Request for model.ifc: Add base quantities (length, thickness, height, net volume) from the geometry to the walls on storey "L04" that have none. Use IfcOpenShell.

First a look at what the model holds.

```python
import ifcopenshell
import ifcopenshell.util.element
import ifcopenshell.util.unit

model = ifcopenshell.open("model.ifc")
print(model.schema)
for unit_type in ("LENGTHUNIT", "AREAUNIT", "VOLUMEUNIT"):
    print(unit_type, ifcopenshell.util.unit.calculate_unit_scale(model, unit_type))
storey = next(s for s in model.by_type("IfcBuildingStorey") if s.Name == "L04")
walls = [e for e in ifcopenshell.util.element.get_decomposition(storey) if e.is_a("IfcWall")]
for e in sorted(walls, key=lambda e: e.id()):
    print(e.id(), e.is_a(), e.Name, list(ifcopenshell.util.element.get_psets(e, qtos_only=True)), sep=" | ")
```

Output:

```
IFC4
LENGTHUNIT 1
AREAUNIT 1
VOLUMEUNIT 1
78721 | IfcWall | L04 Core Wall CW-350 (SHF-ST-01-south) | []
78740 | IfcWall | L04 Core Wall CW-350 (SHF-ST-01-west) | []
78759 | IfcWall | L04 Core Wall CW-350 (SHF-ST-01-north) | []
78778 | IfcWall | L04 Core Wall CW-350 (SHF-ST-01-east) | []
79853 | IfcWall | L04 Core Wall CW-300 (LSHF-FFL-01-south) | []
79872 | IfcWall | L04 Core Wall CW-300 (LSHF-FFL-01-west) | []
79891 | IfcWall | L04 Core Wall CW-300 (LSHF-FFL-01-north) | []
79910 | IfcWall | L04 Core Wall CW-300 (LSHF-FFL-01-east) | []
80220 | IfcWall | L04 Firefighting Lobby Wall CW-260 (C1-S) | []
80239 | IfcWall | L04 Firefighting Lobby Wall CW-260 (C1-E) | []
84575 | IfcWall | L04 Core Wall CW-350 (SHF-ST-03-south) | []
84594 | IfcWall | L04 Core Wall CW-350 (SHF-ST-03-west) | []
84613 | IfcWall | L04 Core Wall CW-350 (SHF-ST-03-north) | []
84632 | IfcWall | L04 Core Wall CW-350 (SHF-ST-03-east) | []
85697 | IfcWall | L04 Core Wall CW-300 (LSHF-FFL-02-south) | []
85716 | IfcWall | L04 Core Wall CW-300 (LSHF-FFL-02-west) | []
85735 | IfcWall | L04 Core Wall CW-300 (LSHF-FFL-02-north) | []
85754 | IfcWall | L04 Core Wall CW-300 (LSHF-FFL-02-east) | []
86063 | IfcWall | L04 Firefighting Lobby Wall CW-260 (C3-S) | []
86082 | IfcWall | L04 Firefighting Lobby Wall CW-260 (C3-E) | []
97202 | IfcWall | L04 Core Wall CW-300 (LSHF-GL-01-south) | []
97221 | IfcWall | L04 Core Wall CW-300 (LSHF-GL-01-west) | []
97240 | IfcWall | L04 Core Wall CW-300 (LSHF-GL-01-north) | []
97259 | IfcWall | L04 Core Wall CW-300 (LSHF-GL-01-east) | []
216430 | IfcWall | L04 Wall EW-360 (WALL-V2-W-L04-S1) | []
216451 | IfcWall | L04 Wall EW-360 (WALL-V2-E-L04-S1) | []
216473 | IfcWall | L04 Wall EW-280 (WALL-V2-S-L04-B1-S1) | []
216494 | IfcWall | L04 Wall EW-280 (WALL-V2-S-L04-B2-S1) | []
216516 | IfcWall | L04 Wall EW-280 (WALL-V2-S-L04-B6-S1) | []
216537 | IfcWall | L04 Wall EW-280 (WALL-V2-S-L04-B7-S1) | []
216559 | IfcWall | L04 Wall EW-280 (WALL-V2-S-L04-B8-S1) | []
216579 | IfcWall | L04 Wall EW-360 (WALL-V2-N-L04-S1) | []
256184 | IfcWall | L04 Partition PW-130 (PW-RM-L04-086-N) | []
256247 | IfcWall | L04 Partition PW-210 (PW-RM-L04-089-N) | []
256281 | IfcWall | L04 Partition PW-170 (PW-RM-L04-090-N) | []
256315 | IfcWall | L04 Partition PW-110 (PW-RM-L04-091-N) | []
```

```python
import ifcopenshell
import ifcopenshell.api.pset
import ifcopenshell.geom
import ifcopenshell.util.element
import ifcopenshell.util.shape
import ifcopenshell.util.unit

model = ifcopenshell.open("model.ifc")
unit_scale = ifcopenshell.util.unit.calculate_unit_scale(model)
volume_scale = ifcopenshell.util.unit.calculate_unit_scale(model, "VOLUMEUNIT")
settings = ifcopenshell.geom.settings()

storey = next(s for s in model.by_type("IfcBuildingStorey") if s.Name == "L04")
walls = [e for e in ifcopenshell.util.element.get_decomposition(storey) if e.is_a("IfcWall")]

for e in sorted(walls, key=lambda e: e.id()):
    if ifcopenshell.util.element.get_psets(e, qtos_only=True, should_inherit=False):
        continue
    # Geometry comes back in metres, in the element's own axes.
    shape = ifcopenshell.geom.create_shape(settings, e)
    values = {
        "Length": ifcopenshell.util.shape.get_x(shape.geometry) / unit_scale,
        "Width": ifcopenshell.util.shape.get_y(shape.geometry) / unit_scale,
        "Height": ifcopenshell.util.shape.get_z(shape.geometry) / unit_scale,
        "NetVolume": ifcopenshell.util.shape.get_volume(shape.geometry) / volume_scale,
    }
    qto = ifcopenshell.api.pset.add_qto(model, product=e, name="Qto_WallBaseQuantities")
    ifcopenshell.api.pset.edit_qto(model, qto=qto, properties=values)
    print(e.id(), {k: round(v, 3) for k, v in values.items()})

model.write("model_rev.ifc")
```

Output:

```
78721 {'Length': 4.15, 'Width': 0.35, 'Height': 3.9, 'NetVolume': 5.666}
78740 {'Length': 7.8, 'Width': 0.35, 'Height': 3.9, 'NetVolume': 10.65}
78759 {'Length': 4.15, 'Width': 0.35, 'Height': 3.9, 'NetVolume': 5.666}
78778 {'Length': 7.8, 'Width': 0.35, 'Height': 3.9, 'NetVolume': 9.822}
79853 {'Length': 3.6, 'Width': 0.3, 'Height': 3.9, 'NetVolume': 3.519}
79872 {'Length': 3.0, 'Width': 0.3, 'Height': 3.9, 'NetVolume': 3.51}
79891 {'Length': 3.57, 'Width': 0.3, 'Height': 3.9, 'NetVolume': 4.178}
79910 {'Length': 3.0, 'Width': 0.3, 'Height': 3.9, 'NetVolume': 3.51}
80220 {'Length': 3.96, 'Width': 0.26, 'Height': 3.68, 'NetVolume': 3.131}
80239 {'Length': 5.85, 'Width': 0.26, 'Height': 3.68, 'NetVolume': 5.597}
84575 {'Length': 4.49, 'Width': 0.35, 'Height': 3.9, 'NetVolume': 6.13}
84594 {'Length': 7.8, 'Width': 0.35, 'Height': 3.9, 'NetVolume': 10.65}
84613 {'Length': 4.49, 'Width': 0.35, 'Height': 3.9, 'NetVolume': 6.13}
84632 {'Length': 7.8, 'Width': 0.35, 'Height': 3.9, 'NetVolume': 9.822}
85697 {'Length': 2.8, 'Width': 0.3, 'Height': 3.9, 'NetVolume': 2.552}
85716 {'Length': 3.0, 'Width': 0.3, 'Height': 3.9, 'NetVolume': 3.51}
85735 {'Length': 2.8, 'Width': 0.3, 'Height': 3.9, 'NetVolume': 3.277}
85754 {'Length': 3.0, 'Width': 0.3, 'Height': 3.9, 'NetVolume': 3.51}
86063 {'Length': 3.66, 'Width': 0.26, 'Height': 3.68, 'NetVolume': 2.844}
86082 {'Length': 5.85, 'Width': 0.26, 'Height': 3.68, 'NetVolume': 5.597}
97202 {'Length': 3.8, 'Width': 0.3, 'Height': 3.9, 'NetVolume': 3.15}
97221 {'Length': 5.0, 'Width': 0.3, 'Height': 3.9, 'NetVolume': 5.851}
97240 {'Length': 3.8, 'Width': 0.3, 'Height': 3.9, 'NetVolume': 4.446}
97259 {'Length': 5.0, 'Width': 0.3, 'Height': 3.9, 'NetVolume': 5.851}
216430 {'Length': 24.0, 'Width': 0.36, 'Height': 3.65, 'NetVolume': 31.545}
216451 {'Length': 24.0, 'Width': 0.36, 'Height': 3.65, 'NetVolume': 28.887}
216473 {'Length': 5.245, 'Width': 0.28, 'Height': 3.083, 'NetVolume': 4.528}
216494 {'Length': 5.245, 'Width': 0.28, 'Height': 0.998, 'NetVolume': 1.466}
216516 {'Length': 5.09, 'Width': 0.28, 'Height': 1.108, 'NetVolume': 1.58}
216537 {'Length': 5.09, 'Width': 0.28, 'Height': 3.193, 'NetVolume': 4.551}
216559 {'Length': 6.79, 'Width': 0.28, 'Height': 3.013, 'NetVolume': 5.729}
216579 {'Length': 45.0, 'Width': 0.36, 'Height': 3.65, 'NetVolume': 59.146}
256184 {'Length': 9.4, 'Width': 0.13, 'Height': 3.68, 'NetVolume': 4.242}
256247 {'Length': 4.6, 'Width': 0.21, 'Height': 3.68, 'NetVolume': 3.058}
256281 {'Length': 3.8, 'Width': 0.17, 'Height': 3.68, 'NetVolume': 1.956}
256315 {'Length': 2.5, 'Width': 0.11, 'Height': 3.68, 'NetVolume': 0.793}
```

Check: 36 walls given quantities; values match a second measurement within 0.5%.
